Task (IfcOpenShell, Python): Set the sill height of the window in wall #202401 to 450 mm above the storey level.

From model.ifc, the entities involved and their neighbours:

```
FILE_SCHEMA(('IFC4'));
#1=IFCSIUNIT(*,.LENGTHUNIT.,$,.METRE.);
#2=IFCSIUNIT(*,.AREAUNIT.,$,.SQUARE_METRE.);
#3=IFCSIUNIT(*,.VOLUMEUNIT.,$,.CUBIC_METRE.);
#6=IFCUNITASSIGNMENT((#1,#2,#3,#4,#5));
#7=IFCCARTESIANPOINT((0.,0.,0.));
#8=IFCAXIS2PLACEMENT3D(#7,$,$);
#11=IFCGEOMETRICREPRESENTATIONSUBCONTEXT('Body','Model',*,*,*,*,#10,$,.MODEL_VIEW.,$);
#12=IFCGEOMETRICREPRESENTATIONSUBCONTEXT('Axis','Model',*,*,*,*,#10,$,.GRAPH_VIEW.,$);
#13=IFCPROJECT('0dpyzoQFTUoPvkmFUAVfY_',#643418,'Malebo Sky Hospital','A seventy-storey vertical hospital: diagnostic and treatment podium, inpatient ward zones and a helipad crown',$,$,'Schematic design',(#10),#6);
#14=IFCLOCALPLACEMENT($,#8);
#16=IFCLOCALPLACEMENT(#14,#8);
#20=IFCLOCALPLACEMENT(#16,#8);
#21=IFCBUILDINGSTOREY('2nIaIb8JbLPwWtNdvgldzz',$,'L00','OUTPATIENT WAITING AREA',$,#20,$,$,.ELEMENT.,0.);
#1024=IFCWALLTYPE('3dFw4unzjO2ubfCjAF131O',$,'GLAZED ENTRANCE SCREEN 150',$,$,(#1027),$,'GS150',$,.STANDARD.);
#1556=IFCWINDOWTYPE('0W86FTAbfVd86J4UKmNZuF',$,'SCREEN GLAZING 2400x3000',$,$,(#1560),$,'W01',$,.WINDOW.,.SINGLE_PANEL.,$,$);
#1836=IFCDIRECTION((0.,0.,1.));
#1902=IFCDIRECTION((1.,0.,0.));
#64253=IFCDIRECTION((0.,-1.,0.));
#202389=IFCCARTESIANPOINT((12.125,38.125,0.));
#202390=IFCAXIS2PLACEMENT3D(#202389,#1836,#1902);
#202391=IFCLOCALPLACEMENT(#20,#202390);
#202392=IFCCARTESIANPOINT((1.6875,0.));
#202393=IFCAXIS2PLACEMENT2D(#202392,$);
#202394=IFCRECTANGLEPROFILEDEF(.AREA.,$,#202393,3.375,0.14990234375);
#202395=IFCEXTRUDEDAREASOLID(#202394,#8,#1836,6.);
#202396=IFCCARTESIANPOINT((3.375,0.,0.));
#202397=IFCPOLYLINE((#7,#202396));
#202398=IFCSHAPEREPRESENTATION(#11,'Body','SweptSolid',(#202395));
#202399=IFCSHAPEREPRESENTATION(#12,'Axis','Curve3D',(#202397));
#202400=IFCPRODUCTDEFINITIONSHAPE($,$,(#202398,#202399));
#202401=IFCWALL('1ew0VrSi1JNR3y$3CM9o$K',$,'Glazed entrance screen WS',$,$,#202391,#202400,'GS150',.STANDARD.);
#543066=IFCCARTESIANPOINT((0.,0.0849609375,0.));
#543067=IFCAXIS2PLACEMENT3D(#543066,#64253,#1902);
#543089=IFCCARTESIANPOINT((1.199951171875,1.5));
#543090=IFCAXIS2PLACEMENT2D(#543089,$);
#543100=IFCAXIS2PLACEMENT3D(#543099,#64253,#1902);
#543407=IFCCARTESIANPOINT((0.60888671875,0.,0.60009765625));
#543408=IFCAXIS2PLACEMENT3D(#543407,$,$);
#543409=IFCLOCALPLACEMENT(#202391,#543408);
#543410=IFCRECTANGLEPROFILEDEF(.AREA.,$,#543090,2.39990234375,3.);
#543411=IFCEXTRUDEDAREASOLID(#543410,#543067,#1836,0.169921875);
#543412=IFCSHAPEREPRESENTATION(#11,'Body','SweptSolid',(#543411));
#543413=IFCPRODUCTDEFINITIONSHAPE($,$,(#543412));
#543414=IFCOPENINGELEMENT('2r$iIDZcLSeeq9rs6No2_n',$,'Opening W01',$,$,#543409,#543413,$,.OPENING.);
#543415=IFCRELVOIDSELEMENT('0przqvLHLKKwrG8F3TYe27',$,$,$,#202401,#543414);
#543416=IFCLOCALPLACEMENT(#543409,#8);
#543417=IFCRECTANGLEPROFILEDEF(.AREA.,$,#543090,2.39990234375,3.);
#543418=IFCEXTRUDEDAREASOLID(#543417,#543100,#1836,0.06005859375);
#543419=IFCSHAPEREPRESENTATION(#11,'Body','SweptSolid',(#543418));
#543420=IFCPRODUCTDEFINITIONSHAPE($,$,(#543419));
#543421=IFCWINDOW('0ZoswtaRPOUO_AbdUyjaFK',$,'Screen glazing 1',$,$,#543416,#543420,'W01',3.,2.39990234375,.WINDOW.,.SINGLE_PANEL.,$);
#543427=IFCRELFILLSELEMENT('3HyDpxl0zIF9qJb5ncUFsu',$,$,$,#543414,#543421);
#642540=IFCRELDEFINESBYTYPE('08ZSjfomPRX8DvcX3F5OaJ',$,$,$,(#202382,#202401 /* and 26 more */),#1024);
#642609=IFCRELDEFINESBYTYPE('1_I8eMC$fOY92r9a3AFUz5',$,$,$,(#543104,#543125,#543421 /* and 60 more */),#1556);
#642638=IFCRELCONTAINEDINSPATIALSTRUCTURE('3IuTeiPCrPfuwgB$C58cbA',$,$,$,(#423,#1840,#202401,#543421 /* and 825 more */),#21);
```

```python
import numpy as np
import ifcopenshell
import ifcopenshell.api.geometry
import ifcopenshell.geom
import ifcopenshell.util.element
import ifcopenshell.util.placement
import ifcopenshell.util.shape
import ifcopenshell.util.unit

model = ifcopenshell.open("model.ifc")
unit_scale = ifcopenshell.util.unit.calculate_unit_scale(model)

window = model.by_guid("0ZoswtaRPOUO_AbdUyjaFK")
opening = window.FillsVoids[0].RelatingOpeningElement
storey = ifcopenshell.util.element.get_container(window, ifc_class="IfcBuildingStorey")
level = ifcopenshell.util.placement.get_local_placement(storey.ObjectPlacement)[2, 3]

# The opening's origin need not be at the sill, so measure its lowest point.
shape = ifcopenshell.geom.create_shape(ifcopenshell.geom.settings(), opening)
bottom = ifcopenshell.util.shape.get_shape_bottom_elevation(shape, shape.geometry) / unit_scale
dz = level + 0.45 - bottom

shift = np.array([0.0, 0.0, dz])
# The window is placed relative to its opening, so it follows when the opening moves.
matrix = ifcopenshell.util.placement.get_local_placement(opening.ObjectPlacement)
matrix[:3, 3] += shift
ifcopenshell.api.geometry.edit_object_placement(
    model, product=opening, matrix=matrix, is_si=False, should_transform_children=True
)

print(f"moved by {dz * unit_scale:+.3f} m")

model.write("model_edited.ifc")
```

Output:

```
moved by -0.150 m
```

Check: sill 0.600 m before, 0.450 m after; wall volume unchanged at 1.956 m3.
